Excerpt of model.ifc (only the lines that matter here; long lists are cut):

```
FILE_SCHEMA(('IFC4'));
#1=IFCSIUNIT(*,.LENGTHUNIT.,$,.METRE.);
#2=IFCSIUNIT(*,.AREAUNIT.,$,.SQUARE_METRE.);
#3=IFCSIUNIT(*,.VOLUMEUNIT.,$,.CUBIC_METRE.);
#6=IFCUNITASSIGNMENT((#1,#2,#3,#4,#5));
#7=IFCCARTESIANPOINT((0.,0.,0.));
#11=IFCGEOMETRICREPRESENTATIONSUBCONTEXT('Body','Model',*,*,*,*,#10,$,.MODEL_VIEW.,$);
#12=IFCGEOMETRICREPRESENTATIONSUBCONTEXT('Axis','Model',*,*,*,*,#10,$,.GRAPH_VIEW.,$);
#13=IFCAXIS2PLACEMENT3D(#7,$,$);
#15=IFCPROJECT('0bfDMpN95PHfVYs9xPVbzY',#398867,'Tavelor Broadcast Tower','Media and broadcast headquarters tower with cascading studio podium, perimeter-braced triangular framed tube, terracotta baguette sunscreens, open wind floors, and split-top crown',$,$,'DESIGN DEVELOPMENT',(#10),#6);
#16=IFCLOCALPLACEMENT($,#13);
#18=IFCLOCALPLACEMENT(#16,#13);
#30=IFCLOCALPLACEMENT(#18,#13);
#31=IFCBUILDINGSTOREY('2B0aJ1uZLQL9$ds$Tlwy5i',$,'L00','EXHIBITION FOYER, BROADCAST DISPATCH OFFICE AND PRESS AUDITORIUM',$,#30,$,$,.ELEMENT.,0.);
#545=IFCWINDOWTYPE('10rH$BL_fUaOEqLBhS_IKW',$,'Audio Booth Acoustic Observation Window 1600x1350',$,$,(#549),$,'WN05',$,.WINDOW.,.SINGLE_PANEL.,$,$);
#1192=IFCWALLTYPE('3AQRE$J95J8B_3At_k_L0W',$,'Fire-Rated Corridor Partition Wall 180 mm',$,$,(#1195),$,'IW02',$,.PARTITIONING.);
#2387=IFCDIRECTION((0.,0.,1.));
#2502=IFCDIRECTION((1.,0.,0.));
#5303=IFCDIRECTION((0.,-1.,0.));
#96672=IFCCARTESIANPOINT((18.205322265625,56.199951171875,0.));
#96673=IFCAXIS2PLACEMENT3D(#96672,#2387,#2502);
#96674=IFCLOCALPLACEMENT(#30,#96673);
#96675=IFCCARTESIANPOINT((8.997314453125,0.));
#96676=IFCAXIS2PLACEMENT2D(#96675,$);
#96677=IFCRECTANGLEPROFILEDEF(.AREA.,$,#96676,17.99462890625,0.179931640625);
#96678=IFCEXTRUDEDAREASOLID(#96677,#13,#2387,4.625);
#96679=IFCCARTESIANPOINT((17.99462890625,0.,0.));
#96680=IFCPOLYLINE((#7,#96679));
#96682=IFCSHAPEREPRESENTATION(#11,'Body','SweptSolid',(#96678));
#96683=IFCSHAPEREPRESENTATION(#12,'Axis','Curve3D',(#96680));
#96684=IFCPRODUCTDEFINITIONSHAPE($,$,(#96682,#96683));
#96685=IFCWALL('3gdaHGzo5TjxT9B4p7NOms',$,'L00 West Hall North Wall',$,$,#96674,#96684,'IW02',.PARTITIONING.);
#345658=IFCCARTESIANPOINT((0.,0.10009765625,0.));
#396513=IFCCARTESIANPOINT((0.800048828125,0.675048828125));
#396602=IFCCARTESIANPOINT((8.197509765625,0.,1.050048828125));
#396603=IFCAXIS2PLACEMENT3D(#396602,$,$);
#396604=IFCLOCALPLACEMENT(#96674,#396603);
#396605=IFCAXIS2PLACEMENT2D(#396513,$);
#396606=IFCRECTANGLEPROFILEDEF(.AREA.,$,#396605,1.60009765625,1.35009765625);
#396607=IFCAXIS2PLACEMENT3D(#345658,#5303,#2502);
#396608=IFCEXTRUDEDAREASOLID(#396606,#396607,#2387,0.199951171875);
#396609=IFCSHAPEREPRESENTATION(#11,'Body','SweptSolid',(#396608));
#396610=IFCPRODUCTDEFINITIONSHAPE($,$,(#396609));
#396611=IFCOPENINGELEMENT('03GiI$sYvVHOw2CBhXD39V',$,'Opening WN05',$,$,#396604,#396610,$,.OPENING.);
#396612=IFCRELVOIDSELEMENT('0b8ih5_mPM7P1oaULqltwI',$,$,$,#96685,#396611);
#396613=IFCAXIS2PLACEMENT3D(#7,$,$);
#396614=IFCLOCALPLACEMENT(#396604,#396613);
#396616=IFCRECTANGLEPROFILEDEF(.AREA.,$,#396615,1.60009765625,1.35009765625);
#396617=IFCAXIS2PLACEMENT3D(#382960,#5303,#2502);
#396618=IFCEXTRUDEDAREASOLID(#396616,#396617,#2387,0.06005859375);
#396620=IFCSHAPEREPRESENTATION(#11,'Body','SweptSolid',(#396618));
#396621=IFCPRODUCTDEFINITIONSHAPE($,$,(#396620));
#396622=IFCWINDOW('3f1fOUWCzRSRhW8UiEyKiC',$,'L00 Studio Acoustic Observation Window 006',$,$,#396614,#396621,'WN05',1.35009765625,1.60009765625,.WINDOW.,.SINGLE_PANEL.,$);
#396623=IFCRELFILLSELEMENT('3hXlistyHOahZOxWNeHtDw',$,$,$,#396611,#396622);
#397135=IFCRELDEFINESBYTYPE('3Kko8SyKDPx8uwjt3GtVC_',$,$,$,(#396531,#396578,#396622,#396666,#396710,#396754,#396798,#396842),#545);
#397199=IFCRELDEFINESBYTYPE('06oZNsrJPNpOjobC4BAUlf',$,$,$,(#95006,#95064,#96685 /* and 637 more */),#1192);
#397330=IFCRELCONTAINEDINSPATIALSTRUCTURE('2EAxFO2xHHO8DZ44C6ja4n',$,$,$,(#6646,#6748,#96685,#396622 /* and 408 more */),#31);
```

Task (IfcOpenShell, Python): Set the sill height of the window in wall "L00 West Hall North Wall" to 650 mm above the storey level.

```python
import numpy as np
import ifcopenshell
import ifcopenshell.api.geometry
import ifcopenshell.geom
import ifcopenshell.util.element
import ifcopenshell.util.placement
import ifcopenshell.util.shape
import ifcopenshell.util.unit

model = ifcopenshell.open("model.ifc")
unit_scale = ifcopenshell.util.unit.calculate_unit_scale(model)

window = model.by_guid("3f1fOUWCzRSRhW8UiEyKiC")
opening = window.FillsVoids[0].RelatingOpeningElement
storey = ifcopenshell.util.element.get_container(window, ifc_class="IfcBuildingStorey")
level = ifcopenshell.util.placement.get_local_placement(storey.ObjectPlacement)[2, 3]

# The opening's origin need not be at the sill, so measure its lowest point.
shape = ifcopenshell.geom.create_shape(ifcopenshell.geom.settings(), opening)
bottom = ifcopenshell.util.shape.get_shape_bottom_elevation(shape, shape.geometry) / unit_scale
dz = level + 0.65 / unit_scale - bottom

shift = np.array([0.0, 0.0, dz])
# The window is placed relative to its opening, so it follows when the opening moves.
matrix = ifcopenshell.util.placement.get_local_placement(opening.ObjectPlacement)
matrix[:3, 3] += shift
ifcopenshell.api.geometry.edit_object_placement(
    model, product=opening, matrix=matrix, is_si=False, should_transform_children=True
)

print(f"moved by {dz * unit_scale:+.3f} m")

model.write("model-out.ifc")
```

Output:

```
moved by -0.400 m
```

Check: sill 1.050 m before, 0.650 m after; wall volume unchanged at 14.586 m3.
